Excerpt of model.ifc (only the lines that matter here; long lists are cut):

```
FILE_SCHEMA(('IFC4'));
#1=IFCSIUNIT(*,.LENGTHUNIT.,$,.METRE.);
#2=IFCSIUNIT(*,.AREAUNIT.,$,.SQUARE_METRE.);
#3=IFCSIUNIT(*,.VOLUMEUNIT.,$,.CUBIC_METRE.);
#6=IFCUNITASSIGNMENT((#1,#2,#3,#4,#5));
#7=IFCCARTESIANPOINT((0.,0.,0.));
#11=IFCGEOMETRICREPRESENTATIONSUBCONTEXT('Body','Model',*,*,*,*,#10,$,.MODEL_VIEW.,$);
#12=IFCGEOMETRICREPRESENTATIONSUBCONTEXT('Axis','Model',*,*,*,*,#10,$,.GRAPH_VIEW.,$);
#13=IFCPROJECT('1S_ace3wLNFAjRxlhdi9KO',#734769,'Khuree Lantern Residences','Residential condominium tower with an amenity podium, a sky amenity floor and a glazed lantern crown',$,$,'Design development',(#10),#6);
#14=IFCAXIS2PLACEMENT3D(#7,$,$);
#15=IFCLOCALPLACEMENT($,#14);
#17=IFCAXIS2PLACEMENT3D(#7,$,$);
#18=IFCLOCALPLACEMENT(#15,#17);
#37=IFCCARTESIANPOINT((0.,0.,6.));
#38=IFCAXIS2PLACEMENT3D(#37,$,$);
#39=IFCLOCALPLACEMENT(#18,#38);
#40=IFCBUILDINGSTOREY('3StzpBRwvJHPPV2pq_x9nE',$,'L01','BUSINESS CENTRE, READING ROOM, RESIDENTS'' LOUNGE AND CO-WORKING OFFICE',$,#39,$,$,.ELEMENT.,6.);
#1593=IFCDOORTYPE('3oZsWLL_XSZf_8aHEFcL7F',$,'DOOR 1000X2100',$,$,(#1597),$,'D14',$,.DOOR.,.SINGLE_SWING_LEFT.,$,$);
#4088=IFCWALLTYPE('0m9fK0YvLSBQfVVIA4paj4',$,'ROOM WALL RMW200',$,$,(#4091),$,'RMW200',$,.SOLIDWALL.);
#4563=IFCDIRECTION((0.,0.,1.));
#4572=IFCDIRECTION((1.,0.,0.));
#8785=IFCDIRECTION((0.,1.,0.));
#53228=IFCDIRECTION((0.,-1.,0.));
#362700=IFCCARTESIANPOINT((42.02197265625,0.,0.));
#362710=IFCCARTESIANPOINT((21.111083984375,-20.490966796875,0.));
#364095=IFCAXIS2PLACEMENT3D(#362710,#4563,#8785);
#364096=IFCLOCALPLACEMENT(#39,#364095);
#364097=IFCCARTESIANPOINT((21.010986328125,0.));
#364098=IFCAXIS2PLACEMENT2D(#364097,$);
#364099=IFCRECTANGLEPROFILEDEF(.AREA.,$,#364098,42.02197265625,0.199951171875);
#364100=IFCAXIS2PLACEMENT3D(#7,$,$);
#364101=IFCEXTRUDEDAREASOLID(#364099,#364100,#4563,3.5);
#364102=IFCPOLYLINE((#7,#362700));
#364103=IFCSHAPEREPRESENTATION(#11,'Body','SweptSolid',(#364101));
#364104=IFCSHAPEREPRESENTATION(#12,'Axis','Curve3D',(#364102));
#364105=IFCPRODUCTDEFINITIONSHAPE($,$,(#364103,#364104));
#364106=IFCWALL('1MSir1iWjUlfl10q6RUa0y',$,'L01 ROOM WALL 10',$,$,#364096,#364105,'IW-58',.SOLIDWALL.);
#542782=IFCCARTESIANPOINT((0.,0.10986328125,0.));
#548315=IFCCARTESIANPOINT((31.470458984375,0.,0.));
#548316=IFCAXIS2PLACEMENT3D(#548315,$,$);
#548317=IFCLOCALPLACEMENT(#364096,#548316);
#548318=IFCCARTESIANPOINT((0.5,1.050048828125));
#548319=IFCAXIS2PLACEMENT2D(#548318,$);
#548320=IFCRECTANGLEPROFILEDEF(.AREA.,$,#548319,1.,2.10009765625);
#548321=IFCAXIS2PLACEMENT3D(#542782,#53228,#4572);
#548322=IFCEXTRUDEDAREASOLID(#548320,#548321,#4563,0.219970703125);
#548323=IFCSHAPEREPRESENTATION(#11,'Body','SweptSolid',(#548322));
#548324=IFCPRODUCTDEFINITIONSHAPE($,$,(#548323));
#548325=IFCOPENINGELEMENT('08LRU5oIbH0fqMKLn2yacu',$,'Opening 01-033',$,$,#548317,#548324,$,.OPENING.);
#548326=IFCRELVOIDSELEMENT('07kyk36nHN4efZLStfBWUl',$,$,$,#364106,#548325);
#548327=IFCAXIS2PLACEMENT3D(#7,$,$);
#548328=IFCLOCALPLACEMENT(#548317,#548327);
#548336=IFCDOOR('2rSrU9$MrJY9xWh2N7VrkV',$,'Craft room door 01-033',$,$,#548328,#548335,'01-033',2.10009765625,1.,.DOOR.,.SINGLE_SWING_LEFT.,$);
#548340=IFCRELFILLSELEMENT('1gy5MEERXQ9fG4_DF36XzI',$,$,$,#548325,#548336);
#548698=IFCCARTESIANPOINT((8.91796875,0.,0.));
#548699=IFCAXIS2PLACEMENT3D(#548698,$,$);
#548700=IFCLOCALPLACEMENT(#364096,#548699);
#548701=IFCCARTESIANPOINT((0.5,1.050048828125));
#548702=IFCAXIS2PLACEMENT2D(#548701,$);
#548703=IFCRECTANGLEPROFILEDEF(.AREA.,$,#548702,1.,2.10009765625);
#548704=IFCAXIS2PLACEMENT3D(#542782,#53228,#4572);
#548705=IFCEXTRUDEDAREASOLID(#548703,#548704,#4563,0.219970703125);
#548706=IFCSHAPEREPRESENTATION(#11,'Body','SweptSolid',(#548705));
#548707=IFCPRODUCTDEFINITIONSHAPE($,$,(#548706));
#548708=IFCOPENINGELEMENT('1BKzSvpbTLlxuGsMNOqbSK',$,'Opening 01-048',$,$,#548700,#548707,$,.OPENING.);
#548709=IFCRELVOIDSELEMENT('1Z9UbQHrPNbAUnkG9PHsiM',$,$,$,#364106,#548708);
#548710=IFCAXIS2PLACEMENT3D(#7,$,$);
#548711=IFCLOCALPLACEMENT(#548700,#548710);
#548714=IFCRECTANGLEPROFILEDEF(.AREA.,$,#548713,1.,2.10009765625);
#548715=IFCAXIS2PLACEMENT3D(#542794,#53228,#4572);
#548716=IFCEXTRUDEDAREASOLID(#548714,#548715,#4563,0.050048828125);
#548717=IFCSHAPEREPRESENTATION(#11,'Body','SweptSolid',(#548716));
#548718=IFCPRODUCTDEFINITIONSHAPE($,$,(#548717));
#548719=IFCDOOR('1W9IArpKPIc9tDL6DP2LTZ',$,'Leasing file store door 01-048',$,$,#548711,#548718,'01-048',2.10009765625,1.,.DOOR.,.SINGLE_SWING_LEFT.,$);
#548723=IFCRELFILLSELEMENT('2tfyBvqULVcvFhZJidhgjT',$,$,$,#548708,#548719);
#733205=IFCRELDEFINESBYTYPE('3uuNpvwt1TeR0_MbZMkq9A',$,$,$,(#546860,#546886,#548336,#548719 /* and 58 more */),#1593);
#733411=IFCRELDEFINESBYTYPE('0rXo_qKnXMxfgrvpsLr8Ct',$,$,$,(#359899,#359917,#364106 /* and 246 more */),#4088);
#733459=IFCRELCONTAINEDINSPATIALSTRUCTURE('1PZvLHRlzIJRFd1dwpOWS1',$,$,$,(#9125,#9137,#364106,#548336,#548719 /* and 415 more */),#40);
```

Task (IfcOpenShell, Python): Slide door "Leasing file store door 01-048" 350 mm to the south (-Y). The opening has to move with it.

```python
import ifcopenshell
import ifcopenshell.api.geometry
import ifcopenshell.util.placement
import ifcopenshell.util.unit

model = ifcopenshell.open("model.ifc")
unit_scale = ifcopenshell.util.unit.calculate_unit_scale(model)

door = model.by_guid("1W9IArpKPIc9tDL6DP2LTZ")
opening = door.FillsVoids[0].RelatingOpeningElement
wall = opening.VoidsElements[0].RelatingBuildingElement

wall_matrix = ifcopenshell.util.placement.get_local_placement(wall.ObjectPlacement)
shift = wall_matrix[:3, 0] * -0.35 / unit_scale
before = ifcopenshell.util.placement.get_local_placement(door.ObjectPlacement)[:3, 3].copy()

# The door is placed relative to its opening, so it follows when the opening moves.
matrix = ifcopenshell.util.placement.get_local_placement(opening.ObjectPlacement)
matrix[:3, 3] += shift
ifcopenshell.api.geometry.edit_object_placement(
    model, product=opening, matrix=matrix, is_si=False, should_transform_children=True
)

after = ifcopenshell.util.placement.get_local_placement(door.ObjectPlacement)[:3, 3]
print("door moved by", (after - before).round(3) + 0.0)

model.write("model_updated.ifc")
```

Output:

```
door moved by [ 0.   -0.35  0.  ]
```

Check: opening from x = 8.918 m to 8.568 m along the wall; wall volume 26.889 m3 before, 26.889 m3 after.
